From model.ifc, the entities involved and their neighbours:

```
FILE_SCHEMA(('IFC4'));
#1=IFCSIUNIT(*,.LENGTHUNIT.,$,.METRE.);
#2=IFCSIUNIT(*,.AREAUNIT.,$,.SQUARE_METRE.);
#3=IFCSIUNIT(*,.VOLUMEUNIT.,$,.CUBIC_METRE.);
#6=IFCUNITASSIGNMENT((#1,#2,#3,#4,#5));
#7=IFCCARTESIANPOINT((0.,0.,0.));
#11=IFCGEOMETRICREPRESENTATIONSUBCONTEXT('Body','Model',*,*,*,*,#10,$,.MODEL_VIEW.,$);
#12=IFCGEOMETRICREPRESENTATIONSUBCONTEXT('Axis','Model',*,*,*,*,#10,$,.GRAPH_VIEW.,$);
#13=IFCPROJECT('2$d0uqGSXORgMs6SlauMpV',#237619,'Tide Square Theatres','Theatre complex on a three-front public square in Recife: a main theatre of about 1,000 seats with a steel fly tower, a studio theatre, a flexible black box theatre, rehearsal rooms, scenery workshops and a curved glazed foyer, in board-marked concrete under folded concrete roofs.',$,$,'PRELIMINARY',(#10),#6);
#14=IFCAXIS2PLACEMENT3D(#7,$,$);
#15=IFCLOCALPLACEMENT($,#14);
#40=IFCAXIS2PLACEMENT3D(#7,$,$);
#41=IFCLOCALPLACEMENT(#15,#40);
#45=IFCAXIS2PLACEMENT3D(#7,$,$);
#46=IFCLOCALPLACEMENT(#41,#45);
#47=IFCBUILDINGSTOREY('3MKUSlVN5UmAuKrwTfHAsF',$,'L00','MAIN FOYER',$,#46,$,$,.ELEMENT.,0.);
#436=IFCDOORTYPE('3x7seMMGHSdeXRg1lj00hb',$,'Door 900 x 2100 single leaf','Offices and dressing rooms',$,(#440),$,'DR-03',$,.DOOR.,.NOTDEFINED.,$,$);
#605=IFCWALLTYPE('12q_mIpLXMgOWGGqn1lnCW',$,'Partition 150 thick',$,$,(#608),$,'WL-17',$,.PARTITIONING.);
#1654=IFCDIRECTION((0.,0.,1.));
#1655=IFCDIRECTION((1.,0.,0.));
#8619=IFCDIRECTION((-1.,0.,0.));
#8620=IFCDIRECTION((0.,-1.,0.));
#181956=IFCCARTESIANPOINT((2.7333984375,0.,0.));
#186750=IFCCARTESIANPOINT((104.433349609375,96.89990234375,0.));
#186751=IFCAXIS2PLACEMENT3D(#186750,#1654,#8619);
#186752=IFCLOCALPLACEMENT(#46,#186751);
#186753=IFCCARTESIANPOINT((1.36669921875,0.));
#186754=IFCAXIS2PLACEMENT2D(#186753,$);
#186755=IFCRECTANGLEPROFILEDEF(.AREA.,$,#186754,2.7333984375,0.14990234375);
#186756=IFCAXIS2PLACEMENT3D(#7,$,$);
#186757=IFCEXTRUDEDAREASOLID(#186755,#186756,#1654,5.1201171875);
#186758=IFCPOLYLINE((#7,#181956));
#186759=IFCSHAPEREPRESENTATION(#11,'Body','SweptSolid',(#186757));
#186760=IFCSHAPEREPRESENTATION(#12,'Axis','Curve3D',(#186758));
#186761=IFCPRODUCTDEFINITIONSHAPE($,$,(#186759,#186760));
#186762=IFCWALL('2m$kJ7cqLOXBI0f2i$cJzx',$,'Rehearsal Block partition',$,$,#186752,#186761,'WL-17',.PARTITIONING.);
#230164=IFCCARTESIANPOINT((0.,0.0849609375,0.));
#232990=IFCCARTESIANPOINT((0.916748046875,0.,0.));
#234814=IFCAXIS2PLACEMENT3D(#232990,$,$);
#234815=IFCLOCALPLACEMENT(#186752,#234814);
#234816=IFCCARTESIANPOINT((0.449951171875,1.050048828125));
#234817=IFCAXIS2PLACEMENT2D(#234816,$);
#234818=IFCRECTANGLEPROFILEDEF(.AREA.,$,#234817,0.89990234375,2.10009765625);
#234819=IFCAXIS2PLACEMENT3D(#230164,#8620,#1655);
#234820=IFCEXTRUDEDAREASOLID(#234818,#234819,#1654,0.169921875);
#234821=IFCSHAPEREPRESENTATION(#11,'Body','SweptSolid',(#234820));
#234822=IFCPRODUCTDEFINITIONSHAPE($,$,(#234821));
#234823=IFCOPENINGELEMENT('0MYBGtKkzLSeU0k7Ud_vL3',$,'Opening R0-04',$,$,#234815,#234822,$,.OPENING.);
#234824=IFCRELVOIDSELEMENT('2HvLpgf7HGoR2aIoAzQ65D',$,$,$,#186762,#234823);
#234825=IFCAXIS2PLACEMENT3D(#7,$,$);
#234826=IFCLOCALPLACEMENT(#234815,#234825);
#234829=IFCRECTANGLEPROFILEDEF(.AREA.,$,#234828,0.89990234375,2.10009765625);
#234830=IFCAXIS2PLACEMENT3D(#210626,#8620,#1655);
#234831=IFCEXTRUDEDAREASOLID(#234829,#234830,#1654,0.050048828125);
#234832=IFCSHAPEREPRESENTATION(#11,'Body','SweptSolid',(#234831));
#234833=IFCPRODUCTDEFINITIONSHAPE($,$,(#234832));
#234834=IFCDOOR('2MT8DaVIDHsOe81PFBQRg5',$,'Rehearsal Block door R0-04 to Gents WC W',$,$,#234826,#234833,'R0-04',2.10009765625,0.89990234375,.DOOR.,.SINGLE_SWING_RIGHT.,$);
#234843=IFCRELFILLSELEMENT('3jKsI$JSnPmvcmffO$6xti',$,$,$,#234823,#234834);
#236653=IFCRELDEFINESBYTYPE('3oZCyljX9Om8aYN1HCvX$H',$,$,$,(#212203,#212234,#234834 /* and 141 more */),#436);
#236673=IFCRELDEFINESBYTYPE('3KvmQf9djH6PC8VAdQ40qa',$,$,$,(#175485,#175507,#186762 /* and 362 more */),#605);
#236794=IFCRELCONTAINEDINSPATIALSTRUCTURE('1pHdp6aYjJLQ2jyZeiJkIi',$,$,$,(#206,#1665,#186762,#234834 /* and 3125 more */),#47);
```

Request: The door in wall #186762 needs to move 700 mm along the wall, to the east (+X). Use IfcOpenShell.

```python
import ifcopenshell
import ifcopenshell.api.geometry
import ifcopenshell.util.placement
import ifcopenshell.util.unit

model = ifcopenshell.open("model.ifc")
unit_scale = ifcopenshell.util.unit.calculate_unit_scale(model)

door = model.by_guid("2MT8DaVIDHsOe81PFBQRg5")
opening = door.FillsVoids[0].RelatingOpeningElement
wall = opening.VoidsElements[0].RelatingBuildingElement

wall_matrix = ifcopenshell.util.placement.get_local_placement(wall.ObjectPlacement)
shift = wall_matrix[:3, 0] * -0.7 / unit_scale
before = ifcopenshell.util.placement.get_local_placement(door.ObjectPlacement)[:3, 3].copy()

# The door is placed relative to its opening, so it follows when the opening moves.
matrix = ifcopenshell.util.placement.get_local_placement(opening.ObjectPlacement)
matrix[:3, 3] += shift
ifcopenshell.api.geometry.edit_object_placement(
    model, product=opening, matrix=matrix, is_si=False, should_transform_children=True
)

after = ifcopenshell.util.placement.get_local_placement(door.ObjectPlacement)[:3, 3]
print("door moved by", (after - before).round(3) + 0.0)

model.write("model_edited.ifc")
```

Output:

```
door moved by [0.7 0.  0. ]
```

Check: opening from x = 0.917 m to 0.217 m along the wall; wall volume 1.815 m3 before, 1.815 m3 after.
